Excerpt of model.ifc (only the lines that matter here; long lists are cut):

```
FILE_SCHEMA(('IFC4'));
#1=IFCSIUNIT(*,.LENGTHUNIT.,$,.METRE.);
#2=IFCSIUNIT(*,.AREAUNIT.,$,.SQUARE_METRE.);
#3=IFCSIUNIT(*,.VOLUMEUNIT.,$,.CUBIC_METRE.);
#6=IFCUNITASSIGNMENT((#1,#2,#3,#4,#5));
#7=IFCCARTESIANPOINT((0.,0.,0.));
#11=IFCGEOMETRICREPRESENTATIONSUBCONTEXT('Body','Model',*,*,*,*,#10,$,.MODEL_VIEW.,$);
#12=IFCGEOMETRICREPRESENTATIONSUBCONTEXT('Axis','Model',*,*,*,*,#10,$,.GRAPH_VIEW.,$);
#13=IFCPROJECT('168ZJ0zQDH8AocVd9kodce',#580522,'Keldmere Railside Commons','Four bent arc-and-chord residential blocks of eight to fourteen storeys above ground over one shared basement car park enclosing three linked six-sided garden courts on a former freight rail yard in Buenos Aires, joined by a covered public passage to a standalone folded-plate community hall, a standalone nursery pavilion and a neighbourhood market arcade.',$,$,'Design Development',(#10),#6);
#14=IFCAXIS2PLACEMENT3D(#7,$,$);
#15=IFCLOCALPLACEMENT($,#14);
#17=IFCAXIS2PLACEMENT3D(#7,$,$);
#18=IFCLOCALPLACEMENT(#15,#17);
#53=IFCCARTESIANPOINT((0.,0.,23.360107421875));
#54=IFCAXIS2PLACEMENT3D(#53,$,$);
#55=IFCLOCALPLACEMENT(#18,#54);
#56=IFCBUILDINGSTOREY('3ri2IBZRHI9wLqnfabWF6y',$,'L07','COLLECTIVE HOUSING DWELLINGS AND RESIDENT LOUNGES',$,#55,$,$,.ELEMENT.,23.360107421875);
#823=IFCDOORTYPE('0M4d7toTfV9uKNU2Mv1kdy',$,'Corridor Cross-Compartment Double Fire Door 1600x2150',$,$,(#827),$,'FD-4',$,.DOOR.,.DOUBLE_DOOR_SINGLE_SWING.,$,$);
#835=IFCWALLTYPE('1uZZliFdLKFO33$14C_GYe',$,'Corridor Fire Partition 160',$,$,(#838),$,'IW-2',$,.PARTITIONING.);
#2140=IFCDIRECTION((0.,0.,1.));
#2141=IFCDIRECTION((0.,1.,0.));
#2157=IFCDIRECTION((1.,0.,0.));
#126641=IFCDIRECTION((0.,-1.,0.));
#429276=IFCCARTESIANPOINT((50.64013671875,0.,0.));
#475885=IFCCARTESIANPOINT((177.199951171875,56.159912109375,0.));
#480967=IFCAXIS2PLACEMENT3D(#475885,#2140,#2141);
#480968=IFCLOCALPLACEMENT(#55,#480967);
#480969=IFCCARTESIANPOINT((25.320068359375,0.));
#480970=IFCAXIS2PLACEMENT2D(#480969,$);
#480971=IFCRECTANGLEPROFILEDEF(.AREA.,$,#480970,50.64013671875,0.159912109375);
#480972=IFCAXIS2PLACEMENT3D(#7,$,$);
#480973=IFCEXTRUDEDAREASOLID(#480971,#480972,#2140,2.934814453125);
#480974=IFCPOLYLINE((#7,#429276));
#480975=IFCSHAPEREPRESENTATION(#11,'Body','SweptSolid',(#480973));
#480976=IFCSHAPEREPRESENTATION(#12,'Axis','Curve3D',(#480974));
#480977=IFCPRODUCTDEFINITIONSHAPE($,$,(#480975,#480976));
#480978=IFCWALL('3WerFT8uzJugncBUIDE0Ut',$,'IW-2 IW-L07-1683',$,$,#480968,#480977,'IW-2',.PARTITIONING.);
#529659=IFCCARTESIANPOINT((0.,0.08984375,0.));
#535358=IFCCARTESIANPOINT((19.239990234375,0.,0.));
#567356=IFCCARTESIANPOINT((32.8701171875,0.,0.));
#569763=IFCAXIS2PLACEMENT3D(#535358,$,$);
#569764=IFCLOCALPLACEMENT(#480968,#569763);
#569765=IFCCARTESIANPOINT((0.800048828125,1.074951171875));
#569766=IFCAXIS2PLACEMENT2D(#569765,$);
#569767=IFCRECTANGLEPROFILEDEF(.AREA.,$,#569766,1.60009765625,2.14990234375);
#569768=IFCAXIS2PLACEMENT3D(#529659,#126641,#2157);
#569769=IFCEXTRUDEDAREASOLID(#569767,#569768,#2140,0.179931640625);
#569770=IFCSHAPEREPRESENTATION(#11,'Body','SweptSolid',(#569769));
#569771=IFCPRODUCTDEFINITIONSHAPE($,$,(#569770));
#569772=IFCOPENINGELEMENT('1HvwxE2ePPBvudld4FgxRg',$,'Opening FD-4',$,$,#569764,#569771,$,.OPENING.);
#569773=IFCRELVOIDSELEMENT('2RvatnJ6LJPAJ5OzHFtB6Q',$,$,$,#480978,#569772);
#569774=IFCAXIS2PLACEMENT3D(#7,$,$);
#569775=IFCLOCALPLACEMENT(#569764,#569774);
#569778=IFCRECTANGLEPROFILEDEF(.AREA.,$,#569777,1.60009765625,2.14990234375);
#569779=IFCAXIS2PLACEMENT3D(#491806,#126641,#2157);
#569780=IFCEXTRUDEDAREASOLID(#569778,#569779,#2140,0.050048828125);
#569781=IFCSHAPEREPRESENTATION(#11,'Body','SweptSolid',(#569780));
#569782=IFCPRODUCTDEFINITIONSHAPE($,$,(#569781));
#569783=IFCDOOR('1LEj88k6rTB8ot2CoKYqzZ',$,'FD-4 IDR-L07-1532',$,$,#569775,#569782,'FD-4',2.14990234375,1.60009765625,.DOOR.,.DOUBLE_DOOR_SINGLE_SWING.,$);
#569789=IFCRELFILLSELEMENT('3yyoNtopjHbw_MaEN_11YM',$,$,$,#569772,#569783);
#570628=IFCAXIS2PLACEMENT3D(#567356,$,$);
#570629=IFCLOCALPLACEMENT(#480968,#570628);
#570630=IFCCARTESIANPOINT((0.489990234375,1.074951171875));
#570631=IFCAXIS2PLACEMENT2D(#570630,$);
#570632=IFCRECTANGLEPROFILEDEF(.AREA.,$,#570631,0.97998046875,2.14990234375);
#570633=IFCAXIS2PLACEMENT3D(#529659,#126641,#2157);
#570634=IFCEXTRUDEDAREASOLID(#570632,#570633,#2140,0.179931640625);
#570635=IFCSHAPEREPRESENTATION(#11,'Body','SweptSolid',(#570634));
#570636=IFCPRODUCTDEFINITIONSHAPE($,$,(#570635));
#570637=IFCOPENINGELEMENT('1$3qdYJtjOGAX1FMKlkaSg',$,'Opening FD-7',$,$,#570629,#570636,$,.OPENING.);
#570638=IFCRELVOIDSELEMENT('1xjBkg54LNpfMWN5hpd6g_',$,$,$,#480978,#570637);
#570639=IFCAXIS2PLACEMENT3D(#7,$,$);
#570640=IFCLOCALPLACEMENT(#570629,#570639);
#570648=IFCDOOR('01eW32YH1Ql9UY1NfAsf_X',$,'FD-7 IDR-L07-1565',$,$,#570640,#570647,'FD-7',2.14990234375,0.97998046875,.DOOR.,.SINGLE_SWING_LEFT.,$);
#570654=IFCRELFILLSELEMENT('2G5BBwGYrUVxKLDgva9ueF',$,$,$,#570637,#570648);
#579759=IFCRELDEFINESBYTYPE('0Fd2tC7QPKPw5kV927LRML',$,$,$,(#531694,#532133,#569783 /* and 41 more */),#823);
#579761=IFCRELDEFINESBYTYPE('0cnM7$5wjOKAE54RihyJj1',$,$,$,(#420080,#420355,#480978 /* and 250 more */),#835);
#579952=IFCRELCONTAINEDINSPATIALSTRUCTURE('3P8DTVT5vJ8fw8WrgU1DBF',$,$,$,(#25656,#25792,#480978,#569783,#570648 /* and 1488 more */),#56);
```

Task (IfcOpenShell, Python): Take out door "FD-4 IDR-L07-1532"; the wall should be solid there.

```python
import ifcopenshell
import ifcopenshell.api.feature
import ifcopenshell.api.root
import ifcopenshell.geom
import ifcopenshell.util.shape

model = ifcopenshell.open("model.ifc")
settings = ifcopenshell.geom.settings()


def volume(element):
    """Net volume in cubic metres, openings subtracted."""
    shape = ifcopenshell.geom.create_shape(settings, element)
    return ifcopenshell.util.shape.get_volume(shape.geometry)


door = model.by_guid("1LEj88k6rTB8ot2CoKYqzZ")
opening = door.FillsVoids[0].RelatingOpeningElement
wall = opening.VoidsElements[0].RelatingBuildingElement
before = volume(wall)

ifcopenshell.api.root.remove_product(model, product=door)
ifcopenshell.api.feature.remove_feature(model, feature=opening)

after = volume(wall)

print(f"wall volume {before:.3f} -> {after:.3f} m3")

model.write("model_rev.ifc")
```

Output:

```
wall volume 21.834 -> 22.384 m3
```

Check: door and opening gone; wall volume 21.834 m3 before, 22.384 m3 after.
